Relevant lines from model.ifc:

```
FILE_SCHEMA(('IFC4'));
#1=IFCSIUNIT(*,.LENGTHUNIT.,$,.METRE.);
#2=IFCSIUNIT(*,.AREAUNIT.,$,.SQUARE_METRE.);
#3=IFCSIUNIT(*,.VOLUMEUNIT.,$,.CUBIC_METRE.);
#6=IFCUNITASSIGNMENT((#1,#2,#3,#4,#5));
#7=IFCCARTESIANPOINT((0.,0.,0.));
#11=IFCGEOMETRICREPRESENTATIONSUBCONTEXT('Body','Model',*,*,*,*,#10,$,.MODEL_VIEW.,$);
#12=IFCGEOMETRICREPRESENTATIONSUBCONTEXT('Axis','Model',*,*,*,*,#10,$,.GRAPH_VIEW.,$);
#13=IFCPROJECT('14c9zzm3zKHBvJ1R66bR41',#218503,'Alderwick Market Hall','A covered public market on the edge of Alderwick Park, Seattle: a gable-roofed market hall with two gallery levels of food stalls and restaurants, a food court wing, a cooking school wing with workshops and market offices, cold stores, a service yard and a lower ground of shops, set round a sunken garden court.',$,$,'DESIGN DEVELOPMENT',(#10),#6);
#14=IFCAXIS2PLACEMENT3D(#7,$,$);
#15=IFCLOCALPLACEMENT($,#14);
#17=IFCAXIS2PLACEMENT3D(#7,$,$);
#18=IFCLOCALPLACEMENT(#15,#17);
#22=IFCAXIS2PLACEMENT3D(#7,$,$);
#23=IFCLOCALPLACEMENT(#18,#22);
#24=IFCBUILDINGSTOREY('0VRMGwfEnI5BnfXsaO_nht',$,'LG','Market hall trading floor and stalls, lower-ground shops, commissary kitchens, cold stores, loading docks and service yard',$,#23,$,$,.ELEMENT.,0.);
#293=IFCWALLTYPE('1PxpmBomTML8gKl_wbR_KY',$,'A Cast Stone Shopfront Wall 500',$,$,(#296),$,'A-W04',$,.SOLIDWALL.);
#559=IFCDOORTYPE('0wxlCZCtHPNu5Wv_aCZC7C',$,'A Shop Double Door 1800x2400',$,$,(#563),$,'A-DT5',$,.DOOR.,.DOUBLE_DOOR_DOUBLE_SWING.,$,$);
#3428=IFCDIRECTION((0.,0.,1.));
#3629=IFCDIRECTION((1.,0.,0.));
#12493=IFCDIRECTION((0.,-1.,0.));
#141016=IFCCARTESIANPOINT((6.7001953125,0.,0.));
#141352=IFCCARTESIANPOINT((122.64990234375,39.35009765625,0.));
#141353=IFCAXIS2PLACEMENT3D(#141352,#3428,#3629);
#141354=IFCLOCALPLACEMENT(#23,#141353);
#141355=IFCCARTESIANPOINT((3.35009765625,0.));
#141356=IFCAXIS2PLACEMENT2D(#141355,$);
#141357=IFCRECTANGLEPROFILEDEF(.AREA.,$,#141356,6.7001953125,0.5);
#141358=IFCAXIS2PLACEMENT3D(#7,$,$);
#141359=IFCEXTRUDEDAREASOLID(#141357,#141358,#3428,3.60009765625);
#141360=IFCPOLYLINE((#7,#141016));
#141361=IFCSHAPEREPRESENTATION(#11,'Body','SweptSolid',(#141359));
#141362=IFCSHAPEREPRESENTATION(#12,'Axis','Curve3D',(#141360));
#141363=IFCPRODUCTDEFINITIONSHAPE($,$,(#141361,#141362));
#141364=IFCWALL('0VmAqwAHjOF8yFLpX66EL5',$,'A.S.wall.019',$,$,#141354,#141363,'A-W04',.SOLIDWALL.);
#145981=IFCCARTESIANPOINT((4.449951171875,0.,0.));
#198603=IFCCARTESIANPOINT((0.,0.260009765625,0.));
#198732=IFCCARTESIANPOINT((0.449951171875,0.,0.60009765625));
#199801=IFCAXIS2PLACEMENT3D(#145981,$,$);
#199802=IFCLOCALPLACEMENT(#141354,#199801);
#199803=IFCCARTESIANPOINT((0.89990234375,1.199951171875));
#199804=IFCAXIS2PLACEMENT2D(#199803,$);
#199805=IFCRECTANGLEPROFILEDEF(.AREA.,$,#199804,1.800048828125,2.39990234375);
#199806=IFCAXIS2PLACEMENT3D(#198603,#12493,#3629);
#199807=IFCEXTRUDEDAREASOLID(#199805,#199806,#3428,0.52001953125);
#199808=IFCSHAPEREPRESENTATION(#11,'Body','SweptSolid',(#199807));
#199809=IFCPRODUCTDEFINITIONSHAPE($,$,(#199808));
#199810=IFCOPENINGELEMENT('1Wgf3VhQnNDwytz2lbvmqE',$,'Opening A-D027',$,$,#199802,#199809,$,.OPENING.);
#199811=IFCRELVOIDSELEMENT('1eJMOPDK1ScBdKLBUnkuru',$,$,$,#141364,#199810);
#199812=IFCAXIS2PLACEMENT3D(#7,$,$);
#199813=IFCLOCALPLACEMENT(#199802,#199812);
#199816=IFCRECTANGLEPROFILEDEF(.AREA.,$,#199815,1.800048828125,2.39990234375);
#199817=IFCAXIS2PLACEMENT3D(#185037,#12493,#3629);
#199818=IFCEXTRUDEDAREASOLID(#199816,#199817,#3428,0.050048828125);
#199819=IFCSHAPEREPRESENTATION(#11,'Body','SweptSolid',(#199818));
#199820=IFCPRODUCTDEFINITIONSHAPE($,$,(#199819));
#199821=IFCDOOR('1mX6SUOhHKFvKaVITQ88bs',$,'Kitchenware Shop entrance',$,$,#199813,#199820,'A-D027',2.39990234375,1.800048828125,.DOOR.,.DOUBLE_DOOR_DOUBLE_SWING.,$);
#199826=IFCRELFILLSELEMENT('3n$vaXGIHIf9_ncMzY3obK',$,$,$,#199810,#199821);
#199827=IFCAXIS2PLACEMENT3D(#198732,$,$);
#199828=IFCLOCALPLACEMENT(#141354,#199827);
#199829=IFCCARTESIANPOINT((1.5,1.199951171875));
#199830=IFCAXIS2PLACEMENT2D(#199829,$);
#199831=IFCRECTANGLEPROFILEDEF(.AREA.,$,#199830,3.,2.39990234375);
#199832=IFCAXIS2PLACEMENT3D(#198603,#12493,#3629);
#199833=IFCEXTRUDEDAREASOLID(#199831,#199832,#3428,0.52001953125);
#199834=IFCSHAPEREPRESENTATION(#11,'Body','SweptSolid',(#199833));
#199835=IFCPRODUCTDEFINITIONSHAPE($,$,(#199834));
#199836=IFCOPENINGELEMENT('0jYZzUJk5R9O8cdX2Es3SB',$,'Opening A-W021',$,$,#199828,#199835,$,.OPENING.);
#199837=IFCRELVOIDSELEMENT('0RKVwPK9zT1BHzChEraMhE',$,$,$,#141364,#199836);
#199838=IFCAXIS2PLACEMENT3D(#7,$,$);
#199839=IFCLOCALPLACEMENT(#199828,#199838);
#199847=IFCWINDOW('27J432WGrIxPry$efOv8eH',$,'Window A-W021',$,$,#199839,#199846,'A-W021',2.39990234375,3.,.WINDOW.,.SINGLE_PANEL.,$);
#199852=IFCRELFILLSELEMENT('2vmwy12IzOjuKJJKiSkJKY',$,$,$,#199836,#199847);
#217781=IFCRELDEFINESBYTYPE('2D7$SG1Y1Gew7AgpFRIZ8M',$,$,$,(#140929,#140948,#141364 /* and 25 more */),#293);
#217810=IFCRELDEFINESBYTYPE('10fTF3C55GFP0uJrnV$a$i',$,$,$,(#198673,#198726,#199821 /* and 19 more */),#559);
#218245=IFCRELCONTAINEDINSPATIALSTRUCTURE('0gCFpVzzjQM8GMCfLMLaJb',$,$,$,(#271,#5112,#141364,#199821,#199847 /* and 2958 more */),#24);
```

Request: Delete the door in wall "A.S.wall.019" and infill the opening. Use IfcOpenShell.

```python
import ifcopenshell
import ifcopenshell.api.feature
import ifcopenshell.api.root
import ifcopenshell.geom
import ifcopenshell.util.shape

model = ifcopenshell.open("model.ifc")
settings = ifcopenshell.geom.settings()


def volume(element):
    """Net volume in cubic metres, openings subtracted."""
    shape = ifcopenshell.geom.create_shape(settings, element)
    return ifcopenshell.util.shape.get_volume(shape.geometry)


door = model.by_guid("1mX6SUOhHKFvKaVITQ88bs")
opening = door.FillsVoids[0].RelatingOpeningElement
wall = opening.VoidsElements[0].RelatingBuildingElement
before = volume(wall)

ifcopenshell.api.root.remove_product(model, product=door)
ifcopenshell.api.feature.remove_feature(model, feature=opening)

after = volume(wall)

print(f"wall volume {before:.3f} -> {after:.3f} m3")

model.write("model_edited.ifc")
```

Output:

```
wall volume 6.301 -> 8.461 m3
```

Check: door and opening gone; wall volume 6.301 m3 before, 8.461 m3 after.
